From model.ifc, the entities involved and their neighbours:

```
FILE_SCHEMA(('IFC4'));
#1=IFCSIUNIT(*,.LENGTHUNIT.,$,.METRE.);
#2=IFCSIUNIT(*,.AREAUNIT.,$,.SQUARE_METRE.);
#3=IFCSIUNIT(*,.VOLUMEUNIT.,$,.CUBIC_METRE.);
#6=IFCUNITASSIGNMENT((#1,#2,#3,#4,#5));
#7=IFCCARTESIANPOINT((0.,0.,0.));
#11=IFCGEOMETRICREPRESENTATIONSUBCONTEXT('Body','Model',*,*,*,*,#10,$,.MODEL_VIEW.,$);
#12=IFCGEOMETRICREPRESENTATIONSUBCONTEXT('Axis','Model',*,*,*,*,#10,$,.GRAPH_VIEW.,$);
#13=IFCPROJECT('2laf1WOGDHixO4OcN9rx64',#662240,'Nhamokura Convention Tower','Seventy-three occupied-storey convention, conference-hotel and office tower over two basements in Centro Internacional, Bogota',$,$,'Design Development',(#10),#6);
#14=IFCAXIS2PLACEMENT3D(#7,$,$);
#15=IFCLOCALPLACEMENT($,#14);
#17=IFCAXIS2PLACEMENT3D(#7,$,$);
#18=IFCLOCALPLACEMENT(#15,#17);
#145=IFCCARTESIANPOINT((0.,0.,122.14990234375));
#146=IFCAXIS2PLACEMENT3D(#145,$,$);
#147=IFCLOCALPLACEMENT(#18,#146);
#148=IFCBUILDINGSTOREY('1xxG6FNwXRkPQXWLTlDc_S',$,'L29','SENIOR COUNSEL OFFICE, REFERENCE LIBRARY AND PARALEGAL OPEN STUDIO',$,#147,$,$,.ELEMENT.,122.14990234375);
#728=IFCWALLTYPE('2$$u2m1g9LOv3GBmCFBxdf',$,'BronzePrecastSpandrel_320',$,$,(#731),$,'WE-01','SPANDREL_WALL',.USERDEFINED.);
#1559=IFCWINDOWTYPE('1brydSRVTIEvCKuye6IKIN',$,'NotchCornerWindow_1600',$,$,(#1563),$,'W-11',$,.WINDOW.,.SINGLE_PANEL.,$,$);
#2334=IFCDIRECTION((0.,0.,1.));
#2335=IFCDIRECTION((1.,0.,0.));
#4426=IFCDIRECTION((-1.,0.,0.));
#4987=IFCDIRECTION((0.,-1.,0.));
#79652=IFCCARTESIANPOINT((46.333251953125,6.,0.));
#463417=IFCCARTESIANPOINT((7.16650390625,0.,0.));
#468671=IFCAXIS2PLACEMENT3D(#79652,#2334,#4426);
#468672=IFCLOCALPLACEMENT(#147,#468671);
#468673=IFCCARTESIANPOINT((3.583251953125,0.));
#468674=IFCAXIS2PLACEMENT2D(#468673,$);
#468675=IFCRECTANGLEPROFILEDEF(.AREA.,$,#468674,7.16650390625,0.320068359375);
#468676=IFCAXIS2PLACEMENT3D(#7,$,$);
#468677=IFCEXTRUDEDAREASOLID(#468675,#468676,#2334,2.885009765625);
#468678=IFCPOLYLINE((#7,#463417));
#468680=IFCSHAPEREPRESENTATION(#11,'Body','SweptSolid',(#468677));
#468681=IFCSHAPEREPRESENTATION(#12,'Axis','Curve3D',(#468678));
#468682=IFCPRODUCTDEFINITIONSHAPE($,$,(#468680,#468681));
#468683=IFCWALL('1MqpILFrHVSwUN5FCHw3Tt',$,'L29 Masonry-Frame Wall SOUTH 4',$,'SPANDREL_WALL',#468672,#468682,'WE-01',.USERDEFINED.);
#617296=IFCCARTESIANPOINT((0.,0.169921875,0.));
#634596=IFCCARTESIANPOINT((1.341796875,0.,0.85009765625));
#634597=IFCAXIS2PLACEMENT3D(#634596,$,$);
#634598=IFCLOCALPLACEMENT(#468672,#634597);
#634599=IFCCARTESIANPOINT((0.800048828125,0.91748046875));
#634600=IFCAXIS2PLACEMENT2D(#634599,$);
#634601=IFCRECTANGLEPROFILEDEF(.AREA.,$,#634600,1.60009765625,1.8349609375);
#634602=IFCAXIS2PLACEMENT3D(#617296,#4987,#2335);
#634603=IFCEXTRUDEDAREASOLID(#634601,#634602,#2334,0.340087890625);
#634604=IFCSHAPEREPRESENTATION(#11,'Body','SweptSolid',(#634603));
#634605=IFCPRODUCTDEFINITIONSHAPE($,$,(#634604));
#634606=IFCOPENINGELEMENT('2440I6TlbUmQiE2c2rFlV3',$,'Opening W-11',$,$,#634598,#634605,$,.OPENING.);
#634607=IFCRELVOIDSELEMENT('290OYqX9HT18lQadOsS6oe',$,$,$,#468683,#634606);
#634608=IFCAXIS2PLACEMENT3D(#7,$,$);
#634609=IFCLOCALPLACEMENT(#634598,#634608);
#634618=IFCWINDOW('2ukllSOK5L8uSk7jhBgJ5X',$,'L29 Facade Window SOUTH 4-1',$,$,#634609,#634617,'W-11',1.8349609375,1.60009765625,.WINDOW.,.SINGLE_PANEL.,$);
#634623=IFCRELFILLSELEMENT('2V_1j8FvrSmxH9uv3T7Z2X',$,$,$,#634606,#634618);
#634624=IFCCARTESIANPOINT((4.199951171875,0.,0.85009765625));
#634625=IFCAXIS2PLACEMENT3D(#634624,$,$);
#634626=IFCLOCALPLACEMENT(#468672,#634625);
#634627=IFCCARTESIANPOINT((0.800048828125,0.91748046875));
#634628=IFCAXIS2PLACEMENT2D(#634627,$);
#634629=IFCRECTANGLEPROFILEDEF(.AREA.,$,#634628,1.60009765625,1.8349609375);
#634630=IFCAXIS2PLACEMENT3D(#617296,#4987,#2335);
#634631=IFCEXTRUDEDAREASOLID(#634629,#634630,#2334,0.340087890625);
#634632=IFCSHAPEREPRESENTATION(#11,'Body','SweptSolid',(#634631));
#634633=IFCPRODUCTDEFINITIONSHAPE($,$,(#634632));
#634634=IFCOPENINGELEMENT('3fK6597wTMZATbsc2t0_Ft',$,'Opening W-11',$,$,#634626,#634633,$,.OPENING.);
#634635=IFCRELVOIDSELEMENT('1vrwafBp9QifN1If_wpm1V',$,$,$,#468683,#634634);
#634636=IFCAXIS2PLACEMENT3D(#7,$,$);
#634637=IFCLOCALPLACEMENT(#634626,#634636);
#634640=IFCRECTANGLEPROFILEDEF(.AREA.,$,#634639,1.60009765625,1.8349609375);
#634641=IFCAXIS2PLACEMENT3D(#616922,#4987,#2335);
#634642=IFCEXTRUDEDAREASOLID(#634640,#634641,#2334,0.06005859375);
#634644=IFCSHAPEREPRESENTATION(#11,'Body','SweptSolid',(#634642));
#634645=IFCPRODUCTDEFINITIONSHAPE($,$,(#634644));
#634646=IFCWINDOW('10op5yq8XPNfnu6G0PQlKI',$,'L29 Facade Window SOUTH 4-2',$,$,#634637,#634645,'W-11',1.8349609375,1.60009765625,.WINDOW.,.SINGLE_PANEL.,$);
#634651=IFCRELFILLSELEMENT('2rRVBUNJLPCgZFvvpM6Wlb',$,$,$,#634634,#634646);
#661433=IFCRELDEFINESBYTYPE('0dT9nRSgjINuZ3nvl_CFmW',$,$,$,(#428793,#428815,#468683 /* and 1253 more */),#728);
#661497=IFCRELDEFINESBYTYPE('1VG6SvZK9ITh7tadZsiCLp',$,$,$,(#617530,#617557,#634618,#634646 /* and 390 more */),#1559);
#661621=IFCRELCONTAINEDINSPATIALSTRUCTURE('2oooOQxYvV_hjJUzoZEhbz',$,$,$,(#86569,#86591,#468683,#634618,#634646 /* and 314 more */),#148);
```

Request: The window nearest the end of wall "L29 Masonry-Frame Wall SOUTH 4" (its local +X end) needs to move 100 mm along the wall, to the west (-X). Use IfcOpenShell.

```python
import ifcopenshell
import ifcopenshell.api.geometry
import ifcopenshell.util.placement
import ifcopenshell.util.unit

model = ifcopenshell.open("model.ifc")
unit_scale = ifcopenshell.util.unit.calculate_unit_scale(model)

window = model.by_id(634646)
opening = window.FillsVoids[0].RelatingOpeningElement
wall = opening.VoidsElements[0].RelatingBuildingElement

wall_matrix = ifcopenshell.util.placement.get_local_placement(wall.ObjectPlacement)
shift = wall_matrix[:3, 0] * 0.1 / unit_scale
before = ifcopenshell.util.placement.get_local_placement(window.ObjectPlacement)[:3, 3].copy()

# The window is placed relative to its opening, so it follows when the opening moves.
matrix = ifcopenshell.util.placement.get_local_placement(opening.ObjectPlacement)
matrix[:3, 3] += shift
ifcopenshell.api.geometry.edit_object_placement(
    model, product=opening, matrix=matrix, is_si=False, should_transform_children=True
)

after = ifcopenshell.util.placement.get_local_placement(window.ObjectPlacement)[:3, 3]
print("window moved by", (after - before).round(3) + 0.0)

model.write("model_v2.ifc")
```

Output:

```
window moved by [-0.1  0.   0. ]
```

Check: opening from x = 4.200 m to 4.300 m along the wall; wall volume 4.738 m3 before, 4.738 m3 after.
